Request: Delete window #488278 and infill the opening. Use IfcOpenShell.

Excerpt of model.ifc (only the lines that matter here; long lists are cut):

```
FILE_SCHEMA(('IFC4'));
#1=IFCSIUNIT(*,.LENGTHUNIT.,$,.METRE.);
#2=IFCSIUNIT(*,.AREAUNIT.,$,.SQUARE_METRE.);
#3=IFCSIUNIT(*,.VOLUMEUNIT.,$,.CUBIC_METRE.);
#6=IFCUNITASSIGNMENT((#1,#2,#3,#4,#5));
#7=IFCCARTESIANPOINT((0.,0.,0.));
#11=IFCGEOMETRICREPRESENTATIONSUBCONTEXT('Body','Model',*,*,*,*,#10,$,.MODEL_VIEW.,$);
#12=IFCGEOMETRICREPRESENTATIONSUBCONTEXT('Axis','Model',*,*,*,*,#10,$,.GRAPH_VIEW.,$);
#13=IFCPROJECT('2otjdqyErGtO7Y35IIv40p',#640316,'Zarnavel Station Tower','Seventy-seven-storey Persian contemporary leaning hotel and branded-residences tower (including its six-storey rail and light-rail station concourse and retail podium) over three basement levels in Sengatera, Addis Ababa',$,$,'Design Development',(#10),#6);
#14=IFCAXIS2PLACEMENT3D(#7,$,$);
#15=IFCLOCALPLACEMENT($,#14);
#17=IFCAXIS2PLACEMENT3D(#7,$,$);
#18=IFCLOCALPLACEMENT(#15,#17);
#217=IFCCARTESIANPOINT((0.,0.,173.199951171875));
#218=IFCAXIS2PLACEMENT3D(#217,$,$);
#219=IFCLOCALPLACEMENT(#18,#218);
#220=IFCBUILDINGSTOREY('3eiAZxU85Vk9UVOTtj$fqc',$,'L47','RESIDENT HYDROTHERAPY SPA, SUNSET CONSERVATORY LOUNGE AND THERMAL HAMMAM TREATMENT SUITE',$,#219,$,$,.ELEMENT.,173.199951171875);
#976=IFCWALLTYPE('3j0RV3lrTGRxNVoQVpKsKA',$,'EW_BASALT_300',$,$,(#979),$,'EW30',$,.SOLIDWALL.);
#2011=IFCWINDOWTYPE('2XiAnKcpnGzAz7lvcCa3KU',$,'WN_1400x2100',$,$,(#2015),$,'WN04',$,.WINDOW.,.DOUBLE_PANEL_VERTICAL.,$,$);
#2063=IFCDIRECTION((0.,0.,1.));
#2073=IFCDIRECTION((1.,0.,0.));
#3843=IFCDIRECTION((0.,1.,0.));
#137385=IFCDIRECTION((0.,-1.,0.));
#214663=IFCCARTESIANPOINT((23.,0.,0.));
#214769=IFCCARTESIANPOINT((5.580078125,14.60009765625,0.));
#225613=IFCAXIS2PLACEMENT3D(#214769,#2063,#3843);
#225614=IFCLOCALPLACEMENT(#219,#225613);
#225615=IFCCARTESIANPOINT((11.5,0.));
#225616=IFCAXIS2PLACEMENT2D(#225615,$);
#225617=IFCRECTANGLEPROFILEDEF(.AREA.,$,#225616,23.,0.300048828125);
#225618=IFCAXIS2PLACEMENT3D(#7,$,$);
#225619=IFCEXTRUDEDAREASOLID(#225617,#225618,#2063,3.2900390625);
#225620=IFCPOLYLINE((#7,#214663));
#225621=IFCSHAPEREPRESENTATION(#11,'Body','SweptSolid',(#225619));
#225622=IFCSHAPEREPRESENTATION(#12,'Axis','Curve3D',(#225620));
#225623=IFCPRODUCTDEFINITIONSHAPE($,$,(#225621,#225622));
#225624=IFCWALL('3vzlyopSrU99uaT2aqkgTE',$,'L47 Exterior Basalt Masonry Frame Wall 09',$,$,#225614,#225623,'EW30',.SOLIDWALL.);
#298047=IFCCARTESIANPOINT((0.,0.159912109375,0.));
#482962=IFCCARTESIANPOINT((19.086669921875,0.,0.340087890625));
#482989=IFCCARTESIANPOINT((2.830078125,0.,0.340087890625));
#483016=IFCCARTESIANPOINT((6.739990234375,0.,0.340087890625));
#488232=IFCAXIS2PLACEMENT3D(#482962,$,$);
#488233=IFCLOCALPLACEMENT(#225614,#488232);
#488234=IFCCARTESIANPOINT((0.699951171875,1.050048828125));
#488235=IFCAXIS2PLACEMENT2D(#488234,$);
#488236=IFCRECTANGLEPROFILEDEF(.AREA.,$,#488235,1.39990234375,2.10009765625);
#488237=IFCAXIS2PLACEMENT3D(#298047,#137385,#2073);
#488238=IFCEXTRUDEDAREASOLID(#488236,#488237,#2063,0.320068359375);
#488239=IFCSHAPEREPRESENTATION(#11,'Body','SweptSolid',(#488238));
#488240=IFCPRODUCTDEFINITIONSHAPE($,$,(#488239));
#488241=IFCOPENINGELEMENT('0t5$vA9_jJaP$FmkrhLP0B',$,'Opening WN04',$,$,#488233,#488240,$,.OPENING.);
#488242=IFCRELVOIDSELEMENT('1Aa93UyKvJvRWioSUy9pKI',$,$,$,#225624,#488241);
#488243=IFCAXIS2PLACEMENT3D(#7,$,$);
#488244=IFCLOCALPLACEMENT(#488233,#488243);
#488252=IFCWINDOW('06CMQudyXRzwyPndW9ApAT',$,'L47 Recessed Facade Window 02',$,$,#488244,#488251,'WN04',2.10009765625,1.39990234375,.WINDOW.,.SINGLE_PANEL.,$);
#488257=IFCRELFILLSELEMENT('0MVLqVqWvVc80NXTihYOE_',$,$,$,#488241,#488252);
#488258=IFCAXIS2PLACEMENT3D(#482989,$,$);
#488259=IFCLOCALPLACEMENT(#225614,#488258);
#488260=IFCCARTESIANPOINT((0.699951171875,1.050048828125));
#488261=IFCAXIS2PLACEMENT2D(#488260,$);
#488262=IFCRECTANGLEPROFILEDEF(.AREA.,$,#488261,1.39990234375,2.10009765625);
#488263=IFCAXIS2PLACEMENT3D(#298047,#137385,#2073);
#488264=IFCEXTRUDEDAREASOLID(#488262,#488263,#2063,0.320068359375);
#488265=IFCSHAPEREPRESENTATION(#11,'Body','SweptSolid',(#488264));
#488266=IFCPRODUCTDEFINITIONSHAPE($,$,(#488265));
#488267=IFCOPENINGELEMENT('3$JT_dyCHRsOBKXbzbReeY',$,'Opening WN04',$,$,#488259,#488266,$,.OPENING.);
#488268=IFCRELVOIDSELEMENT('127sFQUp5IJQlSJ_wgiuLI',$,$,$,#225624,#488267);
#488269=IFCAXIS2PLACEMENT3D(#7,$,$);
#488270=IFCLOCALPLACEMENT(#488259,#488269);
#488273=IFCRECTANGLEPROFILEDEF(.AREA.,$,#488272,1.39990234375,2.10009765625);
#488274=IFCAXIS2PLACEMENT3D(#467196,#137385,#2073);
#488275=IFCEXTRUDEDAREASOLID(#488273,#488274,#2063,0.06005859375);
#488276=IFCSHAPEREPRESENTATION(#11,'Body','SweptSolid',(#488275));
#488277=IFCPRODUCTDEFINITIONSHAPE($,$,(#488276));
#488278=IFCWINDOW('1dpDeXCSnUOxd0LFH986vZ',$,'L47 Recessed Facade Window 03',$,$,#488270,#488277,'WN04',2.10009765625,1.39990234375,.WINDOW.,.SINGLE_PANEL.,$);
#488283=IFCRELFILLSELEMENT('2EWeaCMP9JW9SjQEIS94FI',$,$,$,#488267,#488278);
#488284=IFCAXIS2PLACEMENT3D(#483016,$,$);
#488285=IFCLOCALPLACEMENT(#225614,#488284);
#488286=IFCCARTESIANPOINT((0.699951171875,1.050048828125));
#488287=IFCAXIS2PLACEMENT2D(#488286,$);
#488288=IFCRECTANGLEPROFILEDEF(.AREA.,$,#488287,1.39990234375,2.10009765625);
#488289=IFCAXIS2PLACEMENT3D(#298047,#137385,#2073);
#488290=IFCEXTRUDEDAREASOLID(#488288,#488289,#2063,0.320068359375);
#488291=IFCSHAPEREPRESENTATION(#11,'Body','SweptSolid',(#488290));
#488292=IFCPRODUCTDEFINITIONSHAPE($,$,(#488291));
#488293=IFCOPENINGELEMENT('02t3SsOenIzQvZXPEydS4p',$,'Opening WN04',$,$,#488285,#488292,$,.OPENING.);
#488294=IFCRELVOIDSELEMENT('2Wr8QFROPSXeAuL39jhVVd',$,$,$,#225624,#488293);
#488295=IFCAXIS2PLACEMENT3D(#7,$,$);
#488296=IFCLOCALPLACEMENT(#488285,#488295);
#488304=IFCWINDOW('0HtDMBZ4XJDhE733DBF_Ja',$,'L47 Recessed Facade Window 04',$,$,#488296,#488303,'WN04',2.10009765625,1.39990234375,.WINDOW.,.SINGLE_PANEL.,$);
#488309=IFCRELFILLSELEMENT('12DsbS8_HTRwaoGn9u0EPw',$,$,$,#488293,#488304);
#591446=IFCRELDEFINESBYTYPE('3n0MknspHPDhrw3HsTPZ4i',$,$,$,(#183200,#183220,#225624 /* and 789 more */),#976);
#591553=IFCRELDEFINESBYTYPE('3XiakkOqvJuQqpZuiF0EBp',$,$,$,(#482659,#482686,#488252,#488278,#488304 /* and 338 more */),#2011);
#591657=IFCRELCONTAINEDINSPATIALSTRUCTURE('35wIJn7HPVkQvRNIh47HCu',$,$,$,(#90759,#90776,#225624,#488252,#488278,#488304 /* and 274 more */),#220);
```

```python
import ifcopenshell
import ifcopenshell.api.feature
import ifcopenshell.api.root
import ifcopenshell.geom
import ifcopenshell.util.shape

model = ifcopenshell.open("model.ifc")
settings = ifcopenshell.geom.settings()


def volume(element):
    """Net volume in cubic metres, openings subtracted."""
    shape = ifcopenshell.geom.create_shape(settings, element)
    return ifcopenshell.util.shape.get_volume(shape.geometry)


window = model.by_guid("1dpDeXCSnUOxd0LFH986vZ")
opening = window.FillsVoids[0].RelatingOpeningElement
wall = opening.VoidsElements[0].RelatingBuildingElement
before = volume(wall)

ifcopenshell.api.root.remove_product(model, product=window)
ifcopenshell.api.feature.remove_feature(model, feature=opening)

after = volume(wall)

print(f"wall volume {before:.3f} -> {after:.3f} m3")

model.write("model_edited.ifc")
```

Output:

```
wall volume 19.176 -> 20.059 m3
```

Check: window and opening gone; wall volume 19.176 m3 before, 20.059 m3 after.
